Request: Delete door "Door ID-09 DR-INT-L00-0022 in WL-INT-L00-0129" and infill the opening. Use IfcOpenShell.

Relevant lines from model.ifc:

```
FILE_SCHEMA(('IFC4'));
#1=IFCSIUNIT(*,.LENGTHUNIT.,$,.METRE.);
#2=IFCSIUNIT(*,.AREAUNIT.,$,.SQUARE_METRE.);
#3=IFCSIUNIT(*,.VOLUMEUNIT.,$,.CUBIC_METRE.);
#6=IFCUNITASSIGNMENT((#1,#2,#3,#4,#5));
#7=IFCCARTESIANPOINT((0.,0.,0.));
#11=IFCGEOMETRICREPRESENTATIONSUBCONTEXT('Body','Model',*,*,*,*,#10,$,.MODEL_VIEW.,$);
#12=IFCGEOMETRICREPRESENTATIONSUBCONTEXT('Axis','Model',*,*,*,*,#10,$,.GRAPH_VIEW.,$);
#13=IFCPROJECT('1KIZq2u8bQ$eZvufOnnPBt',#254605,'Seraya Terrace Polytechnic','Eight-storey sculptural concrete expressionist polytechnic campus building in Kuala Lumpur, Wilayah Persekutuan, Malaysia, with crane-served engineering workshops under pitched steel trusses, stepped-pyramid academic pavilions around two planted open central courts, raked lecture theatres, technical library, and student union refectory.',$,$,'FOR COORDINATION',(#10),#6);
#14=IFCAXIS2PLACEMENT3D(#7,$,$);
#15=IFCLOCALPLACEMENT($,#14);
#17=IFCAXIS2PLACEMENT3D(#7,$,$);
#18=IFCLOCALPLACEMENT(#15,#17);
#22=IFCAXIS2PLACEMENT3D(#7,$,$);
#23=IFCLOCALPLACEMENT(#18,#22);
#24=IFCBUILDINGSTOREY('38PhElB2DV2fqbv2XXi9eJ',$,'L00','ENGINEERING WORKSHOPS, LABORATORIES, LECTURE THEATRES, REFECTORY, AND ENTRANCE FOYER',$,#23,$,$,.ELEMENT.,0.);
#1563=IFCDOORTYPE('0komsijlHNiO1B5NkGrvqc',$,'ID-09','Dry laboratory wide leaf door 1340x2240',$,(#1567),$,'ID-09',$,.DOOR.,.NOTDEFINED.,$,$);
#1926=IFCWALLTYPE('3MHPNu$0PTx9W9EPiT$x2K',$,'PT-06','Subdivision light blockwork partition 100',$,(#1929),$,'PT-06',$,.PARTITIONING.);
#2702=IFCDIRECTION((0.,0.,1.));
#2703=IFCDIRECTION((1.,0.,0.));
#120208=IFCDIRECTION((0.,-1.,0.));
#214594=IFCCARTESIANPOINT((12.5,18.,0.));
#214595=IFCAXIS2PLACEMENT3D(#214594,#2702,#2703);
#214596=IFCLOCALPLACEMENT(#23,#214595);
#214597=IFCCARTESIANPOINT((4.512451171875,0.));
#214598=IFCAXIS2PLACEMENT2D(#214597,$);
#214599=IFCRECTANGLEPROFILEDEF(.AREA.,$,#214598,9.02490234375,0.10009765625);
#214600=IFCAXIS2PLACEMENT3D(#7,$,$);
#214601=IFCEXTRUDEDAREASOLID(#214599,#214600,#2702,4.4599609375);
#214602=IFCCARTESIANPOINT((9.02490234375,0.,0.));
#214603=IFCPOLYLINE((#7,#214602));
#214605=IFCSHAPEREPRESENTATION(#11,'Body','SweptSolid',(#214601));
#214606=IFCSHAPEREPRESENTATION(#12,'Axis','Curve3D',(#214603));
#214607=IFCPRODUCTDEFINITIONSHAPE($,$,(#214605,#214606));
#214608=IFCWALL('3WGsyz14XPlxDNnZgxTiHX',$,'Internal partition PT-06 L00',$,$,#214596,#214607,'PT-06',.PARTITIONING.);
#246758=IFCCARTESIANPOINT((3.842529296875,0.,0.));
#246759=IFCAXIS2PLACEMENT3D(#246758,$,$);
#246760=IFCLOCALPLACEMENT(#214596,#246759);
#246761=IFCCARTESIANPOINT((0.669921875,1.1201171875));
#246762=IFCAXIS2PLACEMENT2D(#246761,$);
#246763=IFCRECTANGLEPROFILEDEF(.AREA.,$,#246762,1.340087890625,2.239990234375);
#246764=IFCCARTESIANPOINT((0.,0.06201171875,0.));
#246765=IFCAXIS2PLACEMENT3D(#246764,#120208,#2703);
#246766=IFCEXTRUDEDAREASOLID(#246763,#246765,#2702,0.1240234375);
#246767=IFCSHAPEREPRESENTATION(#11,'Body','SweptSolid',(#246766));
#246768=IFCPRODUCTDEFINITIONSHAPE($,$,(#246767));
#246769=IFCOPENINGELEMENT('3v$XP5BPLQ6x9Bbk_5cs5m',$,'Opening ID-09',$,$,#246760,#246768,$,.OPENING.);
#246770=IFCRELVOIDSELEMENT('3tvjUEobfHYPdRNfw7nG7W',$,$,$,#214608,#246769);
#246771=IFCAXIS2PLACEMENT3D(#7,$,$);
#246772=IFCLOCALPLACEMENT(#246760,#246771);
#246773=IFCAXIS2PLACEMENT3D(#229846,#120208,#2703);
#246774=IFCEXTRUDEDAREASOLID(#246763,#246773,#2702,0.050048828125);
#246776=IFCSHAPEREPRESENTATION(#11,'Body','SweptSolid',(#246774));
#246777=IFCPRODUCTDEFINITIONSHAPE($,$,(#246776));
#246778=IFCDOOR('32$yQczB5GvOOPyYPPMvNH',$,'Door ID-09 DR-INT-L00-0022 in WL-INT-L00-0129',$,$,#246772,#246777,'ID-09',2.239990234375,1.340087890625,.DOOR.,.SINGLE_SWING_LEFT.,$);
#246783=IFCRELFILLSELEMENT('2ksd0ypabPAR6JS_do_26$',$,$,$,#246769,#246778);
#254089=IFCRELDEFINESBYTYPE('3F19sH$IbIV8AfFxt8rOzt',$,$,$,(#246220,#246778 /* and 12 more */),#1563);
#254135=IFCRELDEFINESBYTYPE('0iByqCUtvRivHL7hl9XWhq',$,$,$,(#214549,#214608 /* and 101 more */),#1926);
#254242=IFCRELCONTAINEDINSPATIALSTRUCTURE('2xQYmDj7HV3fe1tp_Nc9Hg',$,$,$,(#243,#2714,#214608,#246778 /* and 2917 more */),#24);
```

```python
import ifcopenshell
import ifcopenshell.api.feature
import ifcopenshell.api.root
import ifcopenshell.geom
import ifcopenshell.util.shape

model = ifcopenshell.open("model.ifc")
settings = ifcopenshell.geom.settings()


def volume(element):
    """Net volume in cubic metres, openings subtracted."""
    shape = ifcopenshell.geom.create_shape(settings, element)
    return ifcopenshell.util.shape.get_volume(shape.geometry)


door = model.by_id(246778)
opening = door.FillsVoids[0].RelatingOpeningElement
wall = opening.VoidsElements[0].RelatingBuildingElement
before = volume(wall)

ifcopenshell.api.root.remove_product(model, product=door)
ifcopenshell.api.feature.remove_feature(model, feature=opening)

after = volume(wall)

print(f"wall volume {before:.3f} -> {after:.3f} m3")

model.write("model_updated.ifc")
```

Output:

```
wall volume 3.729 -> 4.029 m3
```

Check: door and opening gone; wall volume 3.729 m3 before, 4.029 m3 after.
